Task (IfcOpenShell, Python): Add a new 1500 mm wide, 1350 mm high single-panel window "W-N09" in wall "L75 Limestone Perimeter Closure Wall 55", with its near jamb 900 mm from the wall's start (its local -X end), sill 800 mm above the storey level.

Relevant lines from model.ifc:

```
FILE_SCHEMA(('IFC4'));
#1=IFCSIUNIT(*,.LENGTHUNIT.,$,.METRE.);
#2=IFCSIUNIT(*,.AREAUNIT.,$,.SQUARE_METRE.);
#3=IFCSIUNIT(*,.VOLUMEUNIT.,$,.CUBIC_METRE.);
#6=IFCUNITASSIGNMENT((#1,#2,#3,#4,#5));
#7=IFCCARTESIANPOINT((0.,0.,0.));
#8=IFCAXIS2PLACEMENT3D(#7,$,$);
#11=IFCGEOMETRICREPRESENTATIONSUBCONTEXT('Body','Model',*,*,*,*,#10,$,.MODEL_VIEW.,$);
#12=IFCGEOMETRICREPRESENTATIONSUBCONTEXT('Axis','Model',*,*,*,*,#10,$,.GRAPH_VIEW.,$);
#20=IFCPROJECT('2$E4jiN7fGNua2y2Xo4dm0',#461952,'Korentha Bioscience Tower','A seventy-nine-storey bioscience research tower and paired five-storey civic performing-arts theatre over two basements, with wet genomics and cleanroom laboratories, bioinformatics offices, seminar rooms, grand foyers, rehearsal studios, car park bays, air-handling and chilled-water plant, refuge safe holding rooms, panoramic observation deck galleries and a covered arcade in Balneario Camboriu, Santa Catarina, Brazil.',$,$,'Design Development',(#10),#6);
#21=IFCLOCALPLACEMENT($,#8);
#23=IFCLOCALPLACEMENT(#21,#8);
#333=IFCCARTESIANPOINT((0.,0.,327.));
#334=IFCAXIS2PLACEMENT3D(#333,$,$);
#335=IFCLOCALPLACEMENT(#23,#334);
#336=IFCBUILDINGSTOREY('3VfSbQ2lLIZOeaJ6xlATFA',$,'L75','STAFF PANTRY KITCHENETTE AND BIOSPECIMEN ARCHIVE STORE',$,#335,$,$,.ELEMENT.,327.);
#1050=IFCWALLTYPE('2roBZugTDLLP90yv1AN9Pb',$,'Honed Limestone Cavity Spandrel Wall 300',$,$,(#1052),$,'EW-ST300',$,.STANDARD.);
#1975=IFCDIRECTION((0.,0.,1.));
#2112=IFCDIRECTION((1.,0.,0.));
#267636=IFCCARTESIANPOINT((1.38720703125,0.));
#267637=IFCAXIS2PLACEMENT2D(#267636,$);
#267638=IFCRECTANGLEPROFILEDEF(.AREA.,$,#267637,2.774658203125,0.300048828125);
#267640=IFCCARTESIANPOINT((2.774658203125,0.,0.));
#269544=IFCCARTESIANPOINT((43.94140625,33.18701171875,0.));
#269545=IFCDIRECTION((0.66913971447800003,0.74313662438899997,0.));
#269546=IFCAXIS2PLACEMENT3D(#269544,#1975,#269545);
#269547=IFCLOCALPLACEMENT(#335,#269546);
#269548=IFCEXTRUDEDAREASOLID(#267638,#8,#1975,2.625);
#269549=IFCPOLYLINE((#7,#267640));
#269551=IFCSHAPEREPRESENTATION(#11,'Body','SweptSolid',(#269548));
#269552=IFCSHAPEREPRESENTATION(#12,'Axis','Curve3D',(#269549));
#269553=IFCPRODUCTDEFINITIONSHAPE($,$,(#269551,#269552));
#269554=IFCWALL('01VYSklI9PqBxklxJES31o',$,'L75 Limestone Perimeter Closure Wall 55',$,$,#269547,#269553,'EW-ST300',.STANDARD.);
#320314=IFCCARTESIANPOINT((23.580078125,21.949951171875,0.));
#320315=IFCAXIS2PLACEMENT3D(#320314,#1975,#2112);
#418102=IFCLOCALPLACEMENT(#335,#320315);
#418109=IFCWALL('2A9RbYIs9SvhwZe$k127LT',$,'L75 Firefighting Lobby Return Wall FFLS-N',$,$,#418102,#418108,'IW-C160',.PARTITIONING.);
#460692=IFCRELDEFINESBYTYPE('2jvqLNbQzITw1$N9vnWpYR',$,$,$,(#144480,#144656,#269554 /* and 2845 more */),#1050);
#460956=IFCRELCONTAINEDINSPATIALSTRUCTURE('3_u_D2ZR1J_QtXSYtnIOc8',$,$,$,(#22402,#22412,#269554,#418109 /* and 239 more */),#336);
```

```python
import numpy as np
import ifcopenshell
import ifcopenshell.api.feature
import ifcopenshell.api.geometry
import ifcopenshell.api.root
import ifcopenshell.api.spatial
import ifcopenshell.geom
import ifcopenshell.util.element
import ifcopenshell.util.placement
import ifcopenshell.util.representation
import ifcopenshell.util.shape
import ifcopenshell.util.unit

model = ifcopenshell.open("model.ifc")
unit_scale = ifcopenshell.util.unit.calculate_unit_scale(model)
settings = ifcopenshell.geom.settings()


def volume(element):
    """Net volume in cubic metres, openings subtracted."""
    shape = ifcopenshell.geom.create_shape(settings, element)
    return ifcopenshell.util.shape.get_volume(shape.geometry)


wall = model.by_guid("01VYSklI9PqBxklxJES31o")
storey = ifcopenshell.util.element.get_container(wall, ifc_class="IfcBuildingStorey")
context = ifcopenshell.util.representation.get_context(model, "Model", "Body", "MODEL_VIEW")
before = volume(wall)

width, height, from_end, sill = 1.5, 1.35, 0.9, 0.8  # metres

# The wall runs along its own X axis, and the end named is its -X end.
wall_shape = ifcopenshell.geom.create_shape(settings, wall)
x, y, z = ifcopenshell.util.shape.get_vertices(wall_shape.geometry).T
start = x.min() + from_end
face, thickness = float(y.min()), float(y.max() - y.min())
wall_matrix = ifcopenshell.util.placement.get_local_placement(wall.ObjectPlacement)
level = ifcopenshell.util.placement.get_local_placement(storey.ObjectPlacement)[2, 3]


def in_wall(x, y):
    """Placement at x, y metres in the wall's axes, at sill height."""
    matrix = wall_matrix.copy()
    matrix[:, 3] = wall_matrix @ np.array([x / unit_scale, y / unit_scale, 0.0, 1.0])
    matrix[2, 3] = level + sill / unit_scale
    return matrix


# Opening: a box that overshoots both wall faces by 50 mm.
opening = ifcopenshell.api.root.create_entity(model, ifc_class="IfcOpeningElement", predefined_type="OPENING")
box = ifcopenshell.api.geometry.add_wall_representation(
    model, context=context, length=width, height=height, thickness=thickness + 0.1
)
ifcopenshell.api.geometry.assign_representation(model, product=opening, representation=box)
ifcopenshell.api.geometry.edit_object_placement(model, product=opening, matrix=in_wall(start, face - 0.05), is_si=False)
ifcopenshell.api.feature.add_feature(model, feature=opening, element=wall)

window = ifcopenshell.api.root.create_entity(model, ifc_class="IfcWindow", name="W-N09", predefined_type="WINDOW")
window.OverallWidth, window.OverallHeight = width / unit_scale, height / unit_scale
window.PartitioningType = "SINGLE_PANEL"
body = ifcopenshell.api.geometry.add_window_representation(
    model,
    context=context,
    overall_width=window.OverallWidth,
    overall_height=window.OverallHeight,
    partition_type="SINGLE_PANEL",
)
ifcopenshell.api.geometry.assign_representation(model, product=window, representation=body)
ifcopenshell.api.spatial.assign_container(model, products=[window], relating_structure=storey)
ifcopenshell.api.feature.add_filling(model, opening=opening, element=window)

# Centre the window in the wall's thickness.
ifcopenshell.api.geometry.edit_object_placement(model, product=window, matrix=in_wall(start, face), is_si=False)
window_shape = ifcopenshell.geom.create_shape(settings, window)
depth = ifcopenshell.util.shape.get_vertices(window_shape.geometry)[:, 1]
offset = face + thickness / 2 - (depth.min() + depth.max()) / 2
ifcopenshell.api.geometry.edit_object_placement(model, product=window, matrix=in_wall(start, offset), is_si=False)

after = volume(wall)

print(f"wall volume {before:.3f} -> {after:.3f} m3")

model.write("model_rev.ifc")
```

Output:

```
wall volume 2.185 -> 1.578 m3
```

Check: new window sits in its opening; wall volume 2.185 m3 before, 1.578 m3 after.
